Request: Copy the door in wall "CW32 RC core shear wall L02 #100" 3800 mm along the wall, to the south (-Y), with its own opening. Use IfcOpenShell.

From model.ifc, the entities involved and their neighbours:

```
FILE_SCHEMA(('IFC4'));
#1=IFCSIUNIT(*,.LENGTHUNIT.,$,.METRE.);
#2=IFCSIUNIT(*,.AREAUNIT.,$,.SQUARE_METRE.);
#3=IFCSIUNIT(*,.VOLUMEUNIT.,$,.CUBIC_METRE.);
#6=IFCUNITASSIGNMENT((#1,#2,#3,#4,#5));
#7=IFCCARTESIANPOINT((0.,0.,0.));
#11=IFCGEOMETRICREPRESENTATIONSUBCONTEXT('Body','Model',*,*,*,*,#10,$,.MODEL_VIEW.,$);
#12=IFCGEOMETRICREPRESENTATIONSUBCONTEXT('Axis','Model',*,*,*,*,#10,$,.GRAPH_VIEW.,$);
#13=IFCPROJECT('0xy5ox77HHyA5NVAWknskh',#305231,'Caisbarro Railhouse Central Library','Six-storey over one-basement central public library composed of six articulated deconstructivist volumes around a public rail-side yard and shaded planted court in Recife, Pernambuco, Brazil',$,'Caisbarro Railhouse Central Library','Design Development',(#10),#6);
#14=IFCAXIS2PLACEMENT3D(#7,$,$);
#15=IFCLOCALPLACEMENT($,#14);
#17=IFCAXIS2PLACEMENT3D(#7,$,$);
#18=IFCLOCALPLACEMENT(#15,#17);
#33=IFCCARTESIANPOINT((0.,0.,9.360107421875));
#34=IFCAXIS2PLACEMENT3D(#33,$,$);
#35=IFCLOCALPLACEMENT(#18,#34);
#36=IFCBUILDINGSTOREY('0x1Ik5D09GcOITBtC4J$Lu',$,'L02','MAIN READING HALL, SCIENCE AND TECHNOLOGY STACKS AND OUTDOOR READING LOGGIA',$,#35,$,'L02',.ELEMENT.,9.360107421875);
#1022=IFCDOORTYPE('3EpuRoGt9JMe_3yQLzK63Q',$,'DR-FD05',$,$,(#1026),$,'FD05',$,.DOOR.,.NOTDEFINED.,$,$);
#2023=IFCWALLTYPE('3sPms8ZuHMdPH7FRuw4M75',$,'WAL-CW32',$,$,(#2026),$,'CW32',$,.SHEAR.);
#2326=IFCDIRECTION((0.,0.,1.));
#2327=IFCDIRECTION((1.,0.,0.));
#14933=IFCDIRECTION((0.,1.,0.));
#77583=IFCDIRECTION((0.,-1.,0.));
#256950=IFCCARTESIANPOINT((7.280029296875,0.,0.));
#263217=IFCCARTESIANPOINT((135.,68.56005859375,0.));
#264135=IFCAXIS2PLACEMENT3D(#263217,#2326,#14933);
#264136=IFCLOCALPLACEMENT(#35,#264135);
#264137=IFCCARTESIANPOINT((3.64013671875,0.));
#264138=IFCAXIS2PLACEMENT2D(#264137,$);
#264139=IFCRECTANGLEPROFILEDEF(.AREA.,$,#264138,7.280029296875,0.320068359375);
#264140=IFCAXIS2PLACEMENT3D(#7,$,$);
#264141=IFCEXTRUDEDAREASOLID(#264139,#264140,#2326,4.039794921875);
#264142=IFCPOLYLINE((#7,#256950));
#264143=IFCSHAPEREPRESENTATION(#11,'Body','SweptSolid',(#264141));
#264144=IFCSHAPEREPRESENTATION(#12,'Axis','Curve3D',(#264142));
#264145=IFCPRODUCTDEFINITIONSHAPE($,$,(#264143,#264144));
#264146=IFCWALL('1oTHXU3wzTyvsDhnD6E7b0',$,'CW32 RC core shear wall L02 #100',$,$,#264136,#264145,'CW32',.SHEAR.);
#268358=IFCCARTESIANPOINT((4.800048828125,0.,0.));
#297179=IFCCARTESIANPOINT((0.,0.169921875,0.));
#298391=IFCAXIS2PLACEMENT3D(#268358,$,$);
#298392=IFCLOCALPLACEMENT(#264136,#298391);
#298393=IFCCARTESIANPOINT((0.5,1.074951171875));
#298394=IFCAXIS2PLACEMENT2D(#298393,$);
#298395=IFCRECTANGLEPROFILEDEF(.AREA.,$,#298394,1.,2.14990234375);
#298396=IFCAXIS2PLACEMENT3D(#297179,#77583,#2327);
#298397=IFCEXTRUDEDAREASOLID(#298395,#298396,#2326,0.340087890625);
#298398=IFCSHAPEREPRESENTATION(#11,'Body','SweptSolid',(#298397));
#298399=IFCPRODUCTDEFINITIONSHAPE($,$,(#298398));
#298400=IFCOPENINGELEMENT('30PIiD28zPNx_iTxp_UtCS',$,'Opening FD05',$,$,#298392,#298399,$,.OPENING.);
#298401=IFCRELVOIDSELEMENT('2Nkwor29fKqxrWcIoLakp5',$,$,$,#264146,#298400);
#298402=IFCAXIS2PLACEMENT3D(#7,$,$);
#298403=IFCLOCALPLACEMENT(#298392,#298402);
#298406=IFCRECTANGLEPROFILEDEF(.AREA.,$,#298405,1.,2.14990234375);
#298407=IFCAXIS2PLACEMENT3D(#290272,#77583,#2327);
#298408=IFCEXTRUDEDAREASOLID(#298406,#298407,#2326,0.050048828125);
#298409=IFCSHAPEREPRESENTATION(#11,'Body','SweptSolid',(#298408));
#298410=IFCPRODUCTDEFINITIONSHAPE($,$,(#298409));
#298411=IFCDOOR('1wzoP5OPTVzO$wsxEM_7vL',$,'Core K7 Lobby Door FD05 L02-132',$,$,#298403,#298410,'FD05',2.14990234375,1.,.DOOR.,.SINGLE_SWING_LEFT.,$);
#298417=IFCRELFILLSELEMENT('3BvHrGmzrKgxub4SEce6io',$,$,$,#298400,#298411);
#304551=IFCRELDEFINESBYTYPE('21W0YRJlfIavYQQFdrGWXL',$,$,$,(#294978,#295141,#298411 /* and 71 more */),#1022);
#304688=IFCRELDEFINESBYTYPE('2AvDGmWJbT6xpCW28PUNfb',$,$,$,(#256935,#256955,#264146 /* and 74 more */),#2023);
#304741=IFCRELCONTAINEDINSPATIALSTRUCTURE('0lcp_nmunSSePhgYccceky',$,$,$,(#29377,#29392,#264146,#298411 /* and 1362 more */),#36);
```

```python
import ifcopenshell
import ifcopenshell.api.feature
import ifcopenshell.api.geometry
import ifcopenshell.api.root
import ifcopenshell.geom
import ifcopenshell.util.element
import ifcopenshell.util.placement
import ifcopenshell.util.shape
import ifcopenshell.util.unit

model = ifcopenshell.open("model.ifc")
unit_scale = ifcopenshell.util.unit.calculate_unit_scale(model)
settings = ifcopenshell.geom.settings()


def volume(element):
    """Net volume in cubic metres, openings subtracted."""
    shape = ifcopenshell.geom.create_shape(settings, element)
    return ifcopenshell.util.shape.get_volume(shape.geometry)


door = model.by_id(298411)
opening = door.FillsVoids[0].RelatingOpeningElement
wall = opening.VoidsElements[0].RelatingBuildingElement
before = volume(wall)
shift = ifcopenshell.util.placement.get_local_placement(wall.ObjectPlacement)[:3, 0] * -3.8 / unit_scale

# copy_class copies the void relationship, type, container and properties, but no geometry.
new_opening = ifcopenshell.api.root.copy_class(model, product=opening)
new_opening.Representation = ifcopenshell.util.element.copy_deep(
    model, opening.Representation, exclude=["IfcGeometricRepresentationContext", "IfcRepresentationMap"]
)
new_door = ifcopenshell.api.root.copy_class(model, product=door)
new_door.Representation = ifcopenshell.util.element.copy_deep(
    model, door.Representation, exclude=["IfcGeometricRepresentationContext", "IfcRepresentationMap"]
)
new_door.Tag = None
ifcopenshell.api.feature.add_filling(model, opening=new_opening, element=new_door)

for old, new in ((opening, new_opening), (door, new_door)):
    matrix = ifcopenshell.util.placement.get_local_placement(old.ObjectPlacement)
    matrix[:3, 3] += shift
    ifcopenshell.api.geometry.edit_object_placement(model, product=new, matrix=matrix, is_si=False)

after = volume(wall)

print(f"wall volume {before:.3f} -> {after:.3f} m3")

model.write("model_v2.ifc")
```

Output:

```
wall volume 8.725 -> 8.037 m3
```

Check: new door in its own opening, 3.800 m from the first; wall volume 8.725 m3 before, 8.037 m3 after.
